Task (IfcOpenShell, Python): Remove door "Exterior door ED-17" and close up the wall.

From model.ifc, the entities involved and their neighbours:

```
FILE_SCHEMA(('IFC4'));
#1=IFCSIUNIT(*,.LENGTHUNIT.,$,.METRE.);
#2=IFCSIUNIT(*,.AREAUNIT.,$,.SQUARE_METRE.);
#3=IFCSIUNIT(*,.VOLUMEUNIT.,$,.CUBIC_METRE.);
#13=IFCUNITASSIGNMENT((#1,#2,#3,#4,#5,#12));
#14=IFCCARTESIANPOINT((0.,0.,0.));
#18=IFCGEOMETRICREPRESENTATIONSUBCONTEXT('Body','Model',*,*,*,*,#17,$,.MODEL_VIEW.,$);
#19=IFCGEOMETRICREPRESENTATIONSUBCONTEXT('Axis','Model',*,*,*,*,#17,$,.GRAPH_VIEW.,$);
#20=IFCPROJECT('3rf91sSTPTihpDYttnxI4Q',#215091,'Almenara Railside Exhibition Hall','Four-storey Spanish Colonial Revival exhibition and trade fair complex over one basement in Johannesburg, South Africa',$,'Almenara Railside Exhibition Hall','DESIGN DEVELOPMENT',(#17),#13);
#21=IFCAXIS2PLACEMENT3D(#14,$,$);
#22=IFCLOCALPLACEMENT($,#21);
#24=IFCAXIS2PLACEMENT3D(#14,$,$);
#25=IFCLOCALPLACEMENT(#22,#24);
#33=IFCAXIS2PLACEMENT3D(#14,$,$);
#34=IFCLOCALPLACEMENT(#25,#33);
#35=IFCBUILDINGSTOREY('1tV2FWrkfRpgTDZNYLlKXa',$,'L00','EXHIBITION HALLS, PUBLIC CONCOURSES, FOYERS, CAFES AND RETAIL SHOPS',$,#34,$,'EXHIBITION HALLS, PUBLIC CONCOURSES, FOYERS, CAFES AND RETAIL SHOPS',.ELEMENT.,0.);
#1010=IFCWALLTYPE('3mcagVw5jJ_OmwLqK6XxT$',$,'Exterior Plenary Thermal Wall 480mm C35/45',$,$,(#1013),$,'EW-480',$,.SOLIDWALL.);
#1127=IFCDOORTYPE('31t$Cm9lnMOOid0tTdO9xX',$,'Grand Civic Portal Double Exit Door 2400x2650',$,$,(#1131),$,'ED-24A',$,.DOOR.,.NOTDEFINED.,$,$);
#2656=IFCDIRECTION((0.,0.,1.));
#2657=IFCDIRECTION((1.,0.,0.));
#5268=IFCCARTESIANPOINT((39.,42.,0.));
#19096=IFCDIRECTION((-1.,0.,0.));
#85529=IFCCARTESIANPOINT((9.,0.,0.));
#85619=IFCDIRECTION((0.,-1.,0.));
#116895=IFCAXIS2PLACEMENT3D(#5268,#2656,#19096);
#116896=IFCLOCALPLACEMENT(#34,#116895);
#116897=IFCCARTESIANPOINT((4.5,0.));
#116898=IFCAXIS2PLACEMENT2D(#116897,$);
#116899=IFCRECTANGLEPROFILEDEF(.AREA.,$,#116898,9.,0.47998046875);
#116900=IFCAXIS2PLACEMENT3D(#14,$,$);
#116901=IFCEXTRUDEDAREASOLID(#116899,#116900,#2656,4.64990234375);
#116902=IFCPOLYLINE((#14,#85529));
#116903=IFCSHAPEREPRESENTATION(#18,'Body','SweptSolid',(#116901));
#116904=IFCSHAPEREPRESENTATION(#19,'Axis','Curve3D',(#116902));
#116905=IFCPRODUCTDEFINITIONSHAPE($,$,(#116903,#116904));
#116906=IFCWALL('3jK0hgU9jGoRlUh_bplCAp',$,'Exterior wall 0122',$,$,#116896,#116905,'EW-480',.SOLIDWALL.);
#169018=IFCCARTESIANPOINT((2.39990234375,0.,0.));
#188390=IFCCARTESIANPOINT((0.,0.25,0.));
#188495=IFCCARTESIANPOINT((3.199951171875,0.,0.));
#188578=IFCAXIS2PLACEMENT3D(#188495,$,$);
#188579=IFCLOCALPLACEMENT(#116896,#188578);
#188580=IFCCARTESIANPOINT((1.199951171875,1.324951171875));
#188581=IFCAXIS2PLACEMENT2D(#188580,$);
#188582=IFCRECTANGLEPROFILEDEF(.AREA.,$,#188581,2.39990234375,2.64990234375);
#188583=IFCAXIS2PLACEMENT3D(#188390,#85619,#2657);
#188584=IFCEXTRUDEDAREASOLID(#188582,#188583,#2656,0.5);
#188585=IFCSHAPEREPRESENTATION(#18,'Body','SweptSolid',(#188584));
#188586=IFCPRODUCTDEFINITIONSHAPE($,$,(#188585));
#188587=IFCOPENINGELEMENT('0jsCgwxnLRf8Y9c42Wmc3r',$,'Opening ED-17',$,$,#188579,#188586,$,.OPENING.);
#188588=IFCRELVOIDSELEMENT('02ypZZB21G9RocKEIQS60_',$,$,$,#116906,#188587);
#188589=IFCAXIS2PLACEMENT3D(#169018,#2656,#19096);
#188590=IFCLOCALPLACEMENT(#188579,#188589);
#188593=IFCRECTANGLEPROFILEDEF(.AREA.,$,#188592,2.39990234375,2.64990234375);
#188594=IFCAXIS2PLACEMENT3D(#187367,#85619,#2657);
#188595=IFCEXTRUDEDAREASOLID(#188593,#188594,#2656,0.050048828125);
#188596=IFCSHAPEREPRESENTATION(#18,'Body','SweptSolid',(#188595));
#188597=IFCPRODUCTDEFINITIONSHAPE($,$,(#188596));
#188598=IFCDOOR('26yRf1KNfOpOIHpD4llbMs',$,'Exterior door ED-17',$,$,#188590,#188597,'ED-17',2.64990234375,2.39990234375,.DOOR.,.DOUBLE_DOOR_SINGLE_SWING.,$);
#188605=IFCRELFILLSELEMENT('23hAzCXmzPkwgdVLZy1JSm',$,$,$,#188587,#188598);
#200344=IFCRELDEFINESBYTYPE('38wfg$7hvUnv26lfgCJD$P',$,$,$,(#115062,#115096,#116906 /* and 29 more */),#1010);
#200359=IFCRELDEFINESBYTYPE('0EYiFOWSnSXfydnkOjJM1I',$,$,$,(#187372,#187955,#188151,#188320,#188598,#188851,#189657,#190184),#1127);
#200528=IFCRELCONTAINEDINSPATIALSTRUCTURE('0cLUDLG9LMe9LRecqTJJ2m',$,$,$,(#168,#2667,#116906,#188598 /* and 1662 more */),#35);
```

```python
import ifcopenshell
import ifcopenshell.api.feature
import ifcopenshell.api.root
import ifcopenshell.geom
import ifcopenshell.util.shape

model = ifcopenshell.open("model.ifc")
settings = ifcopenshell.geom.settings()


def volume(element):
    """Net volume in cubic metres, openings subtracted."""
    shape = ifcopenshell.geom.create_shape(settings, element)
    return ifcopenshell.util.shape.get_volume(shape.geometry)


door = model.by_id(188598)
opening = door.FillsVoids[0].RelatingOpeningElement
wall = opening.VoidsElements[0].RelatingBuildingElement
before = volume(wall)

ifcopenshell.api.root.remove_product(model, product=door)
ifcopenshell.api.feature.remove_feature(model, feature=opening)

after = volume(wall)

print(f"wall volume {before:.3f} -> {after:.3f} m3")

model.write("model_updated.ifc")
```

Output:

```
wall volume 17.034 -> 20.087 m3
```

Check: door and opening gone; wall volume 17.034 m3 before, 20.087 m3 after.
